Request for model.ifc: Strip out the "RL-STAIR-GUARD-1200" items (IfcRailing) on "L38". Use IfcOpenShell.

First a look at what the model holds.

```python
import ifcopenshell
import ifcopenshell.util.element

model = ifcopenshell.open("model.ifc")
print(model.schema)
storey = next(s for s in model.by_type("IfcBuildingStorey") if s.Name == "L38")
railings = [e for e in ifcopenshell.util.element.get_decomposition(storey) if e.is_a("IfcRailing")]
seen = {}
for e in railings:
    element_type = ifcopenshell.util.element.get_type(e)
    name = element_type.Name if element_type not in (None, e) else None
    seen[name] = seen.get(name, 0) + 1
for name, count in sorted(seen.items(), key=str):
    print(count, "x", name)
```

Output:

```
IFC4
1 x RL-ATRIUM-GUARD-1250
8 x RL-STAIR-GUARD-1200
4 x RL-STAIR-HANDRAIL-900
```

```python
import ifcopenshell
import ifcopenshell.api.root
import ifcopenshell.util.element

model = ifcopenshell.open("model.ifc")

storey = next(s for s in model.by_type("IfcBuildingStorey") if s.Name == "L38")
railings = [e for e in ifcopenshell.util.element.get_decomposition(storey) if e.is_a("IfcRailing")]
targets = [e for e in railings if (t := ifcopenshell.util.element.get_type(e)) not in (None, e) and t.Name == "RL-STAIR-GUARD-1200"]

for e in targets:
    ifcopenshell.api.root.remove_product(model, product=e)
print(len(targets), "removed")

model.write("model-out.ifc")
```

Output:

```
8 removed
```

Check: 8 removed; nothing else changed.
